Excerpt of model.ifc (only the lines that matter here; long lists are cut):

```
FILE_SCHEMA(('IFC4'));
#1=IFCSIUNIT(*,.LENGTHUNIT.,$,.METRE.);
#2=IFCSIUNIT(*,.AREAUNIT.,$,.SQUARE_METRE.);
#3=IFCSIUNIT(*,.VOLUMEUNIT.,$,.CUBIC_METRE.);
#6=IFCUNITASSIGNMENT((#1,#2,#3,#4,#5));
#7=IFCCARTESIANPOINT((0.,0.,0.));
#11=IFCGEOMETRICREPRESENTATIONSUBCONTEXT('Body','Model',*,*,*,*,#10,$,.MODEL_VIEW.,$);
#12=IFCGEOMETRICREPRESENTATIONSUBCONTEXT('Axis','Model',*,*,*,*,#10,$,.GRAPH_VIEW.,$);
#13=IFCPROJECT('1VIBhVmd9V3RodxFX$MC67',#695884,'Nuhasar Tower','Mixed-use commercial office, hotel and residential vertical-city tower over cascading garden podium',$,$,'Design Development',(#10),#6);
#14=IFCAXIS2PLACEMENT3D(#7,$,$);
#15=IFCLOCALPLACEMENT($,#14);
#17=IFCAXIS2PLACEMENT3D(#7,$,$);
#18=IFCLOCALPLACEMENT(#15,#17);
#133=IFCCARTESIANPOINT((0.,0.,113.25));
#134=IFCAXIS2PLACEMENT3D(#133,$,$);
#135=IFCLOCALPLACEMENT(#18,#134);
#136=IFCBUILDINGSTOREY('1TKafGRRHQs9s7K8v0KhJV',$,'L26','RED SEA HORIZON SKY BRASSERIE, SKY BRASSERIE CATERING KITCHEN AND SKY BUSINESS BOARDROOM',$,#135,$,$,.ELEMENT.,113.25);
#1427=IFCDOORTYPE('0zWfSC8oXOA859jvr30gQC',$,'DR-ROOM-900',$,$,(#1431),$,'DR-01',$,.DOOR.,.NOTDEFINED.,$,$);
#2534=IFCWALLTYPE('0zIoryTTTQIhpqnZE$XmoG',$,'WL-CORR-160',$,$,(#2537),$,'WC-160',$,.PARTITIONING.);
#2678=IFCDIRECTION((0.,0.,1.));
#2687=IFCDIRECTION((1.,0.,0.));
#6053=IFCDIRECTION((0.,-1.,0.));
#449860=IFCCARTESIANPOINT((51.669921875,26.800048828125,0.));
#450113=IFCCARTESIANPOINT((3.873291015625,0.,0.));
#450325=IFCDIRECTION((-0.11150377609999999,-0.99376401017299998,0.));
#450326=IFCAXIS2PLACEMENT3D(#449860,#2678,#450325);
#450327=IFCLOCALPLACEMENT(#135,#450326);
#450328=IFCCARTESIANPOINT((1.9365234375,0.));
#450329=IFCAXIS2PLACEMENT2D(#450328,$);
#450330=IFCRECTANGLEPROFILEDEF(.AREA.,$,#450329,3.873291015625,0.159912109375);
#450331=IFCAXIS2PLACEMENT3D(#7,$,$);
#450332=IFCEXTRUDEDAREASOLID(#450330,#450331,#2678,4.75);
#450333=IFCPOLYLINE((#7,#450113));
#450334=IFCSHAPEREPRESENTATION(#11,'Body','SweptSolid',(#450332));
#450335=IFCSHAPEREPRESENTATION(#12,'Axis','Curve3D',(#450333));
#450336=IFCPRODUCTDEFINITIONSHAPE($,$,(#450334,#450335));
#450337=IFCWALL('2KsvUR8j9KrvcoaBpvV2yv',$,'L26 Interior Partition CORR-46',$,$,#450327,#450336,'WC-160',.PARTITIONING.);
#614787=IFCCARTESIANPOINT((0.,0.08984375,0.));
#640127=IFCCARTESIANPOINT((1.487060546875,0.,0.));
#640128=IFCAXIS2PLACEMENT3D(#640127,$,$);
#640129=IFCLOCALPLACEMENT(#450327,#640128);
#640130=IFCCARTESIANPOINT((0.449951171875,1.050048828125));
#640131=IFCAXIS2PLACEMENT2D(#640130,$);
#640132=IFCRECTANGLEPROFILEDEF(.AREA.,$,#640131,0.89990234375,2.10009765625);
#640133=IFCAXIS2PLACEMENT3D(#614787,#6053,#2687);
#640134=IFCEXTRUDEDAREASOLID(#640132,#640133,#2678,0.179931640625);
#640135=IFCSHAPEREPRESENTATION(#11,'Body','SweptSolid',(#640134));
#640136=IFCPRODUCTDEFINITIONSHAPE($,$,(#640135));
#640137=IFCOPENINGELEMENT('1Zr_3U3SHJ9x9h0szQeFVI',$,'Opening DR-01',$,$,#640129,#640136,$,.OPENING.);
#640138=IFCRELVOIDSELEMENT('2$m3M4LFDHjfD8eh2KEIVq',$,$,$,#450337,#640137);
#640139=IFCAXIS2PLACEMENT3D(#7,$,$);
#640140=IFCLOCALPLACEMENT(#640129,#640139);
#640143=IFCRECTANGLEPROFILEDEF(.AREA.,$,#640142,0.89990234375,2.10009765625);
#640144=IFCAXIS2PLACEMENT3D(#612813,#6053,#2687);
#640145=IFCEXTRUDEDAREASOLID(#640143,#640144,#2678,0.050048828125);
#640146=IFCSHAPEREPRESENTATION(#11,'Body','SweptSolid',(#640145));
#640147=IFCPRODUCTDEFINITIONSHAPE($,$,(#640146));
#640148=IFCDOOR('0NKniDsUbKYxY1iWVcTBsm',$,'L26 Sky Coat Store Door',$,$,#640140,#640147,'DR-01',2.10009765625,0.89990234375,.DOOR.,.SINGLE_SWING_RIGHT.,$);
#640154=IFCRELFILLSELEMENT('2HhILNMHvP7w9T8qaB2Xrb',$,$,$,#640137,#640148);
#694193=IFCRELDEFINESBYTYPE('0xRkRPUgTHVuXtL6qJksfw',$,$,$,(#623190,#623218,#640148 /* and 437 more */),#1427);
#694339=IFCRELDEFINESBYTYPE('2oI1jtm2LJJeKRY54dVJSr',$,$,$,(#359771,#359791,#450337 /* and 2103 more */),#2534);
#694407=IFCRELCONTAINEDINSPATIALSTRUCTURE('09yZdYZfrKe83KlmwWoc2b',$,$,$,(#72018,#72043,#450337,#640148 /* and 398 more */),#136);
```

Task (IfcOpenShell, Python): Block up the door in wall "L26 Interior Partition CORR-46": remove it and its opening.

```python
import ifcopenshell
import ifcopenshell.api.feature
import ifcopenshell.api.root
import ifcopenshell.geom
import ifcopenshell.util.shape

model = ifcopenshell.open("model.ifc")
settings = ifcopenshell.geom.settings()


def volume(element):
    """Net volume in cubic metres, openings subtracted."""
    shape = ifcopenshell.geom.create_shape(settings, element)
    return ifcopenshell.util.shape.get_volume(shape.geometry)


door = model.by_id(640148)
opening = door.FillsVoids[0].RelatingOpeningElement
wall = opening.VoidsElements[0].RelatingBuildingElement
before = volume(wall)

ifcopenshell.api.root.remove_product(model, product=door)
ifcopenshell.api.feature.remove_feature(model, feature=opening)

after = volume(wall)

print(f"wall volume {before:.3f} -> {after:.3f} m3")

model.write("model_v2.ifc")
```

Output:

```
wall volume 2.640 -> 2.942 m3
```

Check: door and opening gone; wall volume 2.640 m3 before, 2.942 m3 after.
